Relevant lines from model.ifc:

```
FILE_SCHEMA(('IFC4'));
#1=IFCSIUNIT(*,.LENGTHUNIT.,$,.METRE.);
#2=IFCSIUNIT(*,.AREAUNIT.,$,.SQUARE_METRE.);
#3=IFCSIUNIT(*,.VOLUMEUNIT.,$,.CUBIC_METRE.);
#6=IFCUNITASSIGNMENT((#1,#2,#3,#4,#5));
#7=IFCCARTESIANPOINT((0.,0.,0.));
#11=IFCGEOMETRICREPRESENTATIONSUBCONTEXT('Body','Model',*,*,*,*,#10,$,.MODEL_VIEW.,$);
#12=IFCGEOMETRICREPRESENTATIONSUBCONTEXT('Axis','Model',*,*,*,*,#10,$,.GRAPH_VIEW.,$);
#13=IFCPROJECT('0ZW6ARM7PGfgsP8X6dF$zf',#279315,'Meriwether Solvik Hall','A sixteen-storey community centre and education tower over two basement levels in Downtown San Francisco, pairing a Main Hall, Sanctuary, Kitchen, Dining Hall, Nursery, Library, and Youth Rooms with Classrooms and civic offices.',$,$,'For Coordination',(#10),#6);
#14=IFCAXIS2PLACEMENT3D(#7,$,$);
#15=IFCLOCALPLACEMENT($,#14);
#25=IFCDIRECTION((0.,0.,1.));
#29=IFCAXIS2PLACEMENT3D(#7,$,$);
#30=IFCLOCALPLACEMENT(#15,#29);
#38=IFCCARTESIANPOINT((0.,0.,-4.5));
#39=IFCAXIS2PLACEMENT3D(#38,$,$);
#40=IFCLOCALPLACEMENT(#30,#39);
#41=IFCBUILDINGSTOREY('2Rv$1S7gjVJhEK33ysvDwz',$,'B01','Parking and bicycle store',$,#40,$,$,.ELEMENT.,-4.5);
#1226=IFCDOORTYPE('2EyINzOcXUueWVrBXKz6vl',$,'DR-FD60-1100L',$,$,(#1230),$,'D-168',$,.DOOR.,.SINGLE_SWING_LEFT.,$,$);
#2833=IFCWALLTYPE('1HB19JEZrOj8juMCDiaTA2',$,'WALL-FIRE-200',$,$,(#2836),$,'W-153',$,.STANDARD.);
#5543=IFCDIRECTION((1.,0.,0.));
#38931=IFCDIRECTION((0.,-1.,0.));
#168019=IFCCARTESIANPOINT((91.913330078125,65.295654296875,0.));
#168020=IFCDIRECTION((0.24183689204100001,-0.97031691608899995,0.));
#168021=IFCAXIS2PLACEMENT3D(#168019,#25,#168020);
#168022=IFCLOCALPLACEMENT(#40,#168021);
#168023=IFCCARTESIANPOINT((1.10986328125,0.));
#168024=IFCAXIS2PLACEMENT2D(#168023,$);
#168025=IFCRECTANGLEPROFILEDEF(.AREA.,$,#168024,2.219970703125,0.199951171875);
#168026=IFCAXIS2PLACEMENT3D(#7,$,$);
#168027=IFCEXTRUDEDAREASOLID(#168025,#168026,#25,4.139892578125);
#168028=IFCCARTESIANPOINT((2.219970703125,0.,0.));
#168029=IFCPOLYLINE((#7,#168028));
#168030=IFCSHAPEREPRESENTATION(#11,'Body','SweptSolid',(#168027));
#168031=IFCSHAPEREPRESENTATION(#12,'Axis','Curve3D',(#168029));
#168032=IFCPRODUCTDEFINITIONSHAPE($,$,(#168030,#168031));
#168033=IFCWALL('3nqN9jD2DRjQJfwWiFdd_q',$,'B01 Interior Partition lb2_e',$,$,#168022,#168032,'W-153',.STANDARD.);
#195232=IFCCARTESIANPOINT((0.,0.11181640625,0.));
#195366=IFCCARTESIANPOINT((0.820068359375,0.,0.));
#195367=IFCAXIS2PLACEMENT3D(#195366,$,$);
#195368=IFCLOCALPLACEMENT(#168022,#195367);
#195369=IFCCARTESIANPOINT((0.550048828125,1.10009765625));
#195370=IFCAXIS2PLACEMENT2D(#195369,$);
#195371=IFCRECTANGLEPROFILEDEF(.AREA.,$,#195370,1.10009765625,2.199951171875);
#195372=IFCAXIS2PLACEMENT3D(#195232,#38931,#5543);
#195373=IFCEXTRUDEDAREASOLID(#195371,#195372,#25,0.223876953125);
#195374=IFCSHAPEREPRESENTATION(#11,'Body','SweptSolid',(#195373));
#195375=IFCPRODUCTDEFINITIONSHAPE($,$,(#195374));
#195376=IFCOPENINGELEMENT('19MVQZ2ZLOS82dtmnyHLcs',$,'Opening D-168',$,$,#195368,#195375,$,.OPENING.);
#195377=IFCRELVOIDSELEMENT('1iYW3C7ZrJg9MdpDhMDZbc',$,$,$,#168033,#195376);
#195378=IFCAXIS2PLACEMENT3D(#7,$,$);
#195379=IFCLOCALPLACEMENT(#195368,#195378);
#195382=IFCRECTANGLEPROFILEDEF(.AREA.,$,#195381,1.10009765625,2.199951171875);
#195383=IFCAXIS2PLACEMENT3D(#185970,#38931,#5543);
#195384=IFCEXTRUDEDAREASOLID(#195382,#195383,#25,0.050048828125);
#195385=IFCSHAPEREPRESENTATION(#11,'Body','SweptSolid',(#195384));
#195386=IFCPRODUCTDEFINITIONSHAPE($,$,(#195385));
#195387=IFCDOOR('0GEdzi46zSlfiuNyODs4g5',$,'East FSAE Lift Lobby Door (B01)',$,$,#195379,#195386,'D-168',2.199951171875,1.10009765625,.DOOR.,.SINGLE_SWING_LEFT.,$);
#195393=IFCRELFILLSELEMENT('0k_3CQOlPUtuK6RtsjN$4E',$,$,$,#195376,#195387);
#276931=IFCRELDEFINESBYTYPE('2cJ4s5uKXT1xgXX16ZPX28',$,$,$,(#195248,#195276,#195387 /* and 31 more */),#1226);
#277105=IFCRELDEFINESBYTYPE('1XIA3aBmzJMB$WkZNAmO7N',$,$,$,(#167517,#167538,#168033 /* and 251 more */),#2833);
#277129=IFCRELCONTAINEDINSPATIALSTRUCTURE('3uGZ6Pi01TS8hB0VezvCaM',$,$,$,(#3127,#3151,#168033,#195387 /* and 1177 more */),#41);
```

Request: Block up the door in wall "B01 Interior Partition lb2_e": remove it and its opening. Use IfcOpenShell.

```python
import ifcopenshell
import ifcopenshell.api.feature
import ifcopenshell.api.root
import ifcopenshell.geom
import ifcopenshell.util.shape

model = ifcopenshell.open("model.ifc")
settings = ifcopenshell.geom.settings()


def volume(element):
    """Net volume in cubic metres, openings subtracted."""
    shape = ifcopenshell.geom.create_shape(settings, element)
    return ifcopenshell.util.shape.get_volume(shape.geometry)


door = model.by_guid("0GEdzi46zSlfiuNyODs4g5")
opening = door.FillsVoids[0].RelatingOpeningElement
wall = opening.VoidsElements[0].RelatingBuildingElement
before = volume(wall)

ifcopenshell.api.root.remove_product(model, product=door)
ifcopenshell.api.feature.remove_feature(model, feature=opening)

after = volume(wall)

print(f"wall volume {before:.3f} -> {after:.3f} m3")

model.write("model_v2.ifc")
```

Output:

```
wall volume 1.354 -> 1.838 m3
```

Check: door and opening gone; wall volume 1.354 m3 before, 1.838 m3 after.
